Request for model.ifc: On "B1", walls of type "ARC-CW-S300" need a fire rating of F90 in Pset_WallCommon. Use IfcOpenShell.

First a look at what the model holds.

```python
import ifcopenshell
import ifcopenshell.util.element

model = ifcopenshell.open("model.ifc")
print(model.schema)
storey = next(s for s in model.by_type("IfcBuildingStorey") if s.Name == "B1")
walls = [e for e in ifcopenshell.util.element.get_decomposition(storey) if e.is_a("IfcWall")]
seen = {}
for e in walls:
    element_type = ifcopenshell.util.element.get_type(e)
    key = (element_type.Name if element_type != e and element_type else None, ifcopenshell.util.element.get_pset(e, "Pset_WallCommon", "FireRating"))
    seen[key] = seen.get(key, 0) + 1
for (name, value), count in sorted(seen.items(), key=str):
    print(count, "x", name, "|", value)
```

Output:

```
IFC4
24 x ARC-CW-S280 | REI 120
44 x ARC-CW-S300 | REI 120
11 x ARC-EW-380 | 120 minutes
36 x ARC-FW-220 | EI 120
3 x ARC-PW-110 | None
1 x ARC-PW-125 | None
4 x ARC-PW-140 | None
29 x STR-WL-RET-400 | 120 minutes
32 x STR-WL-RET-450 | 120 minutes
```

```python
import ifcopenshell
import ifcopenshell.api.pset
import ifcopenshell.util.element

model = ifcopenshell.open("model.ifc")

storey = next(s for s in model.by_type("IfcBuildingStorey") if s.Name == "B1")
walls = [e for e in ifcopenshell.util.element.get_decomposition(storey) if e.is_a("IfcWall")]

count = 0
for e in walls:
    element_type = ifcopenshell.util.element.get_type(e)
    if element_type in (None, e) or element_type.Name != "ARC-CW-S300":
        continue
    # add_pset returns the element's existing set when there is one.
    pset = ifcopenshell.api.pset.add_pset(model, product=e, name="Pset_WallCommon")
    ifcopenshell.api.pset.edit_pset(model, pset=pset, properties={"FireRating": "F90"})
    count += 1

print(count, "walls updated")

model.write("model_v2.ifc")
```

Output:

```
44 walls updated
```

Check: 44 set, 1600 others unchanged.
